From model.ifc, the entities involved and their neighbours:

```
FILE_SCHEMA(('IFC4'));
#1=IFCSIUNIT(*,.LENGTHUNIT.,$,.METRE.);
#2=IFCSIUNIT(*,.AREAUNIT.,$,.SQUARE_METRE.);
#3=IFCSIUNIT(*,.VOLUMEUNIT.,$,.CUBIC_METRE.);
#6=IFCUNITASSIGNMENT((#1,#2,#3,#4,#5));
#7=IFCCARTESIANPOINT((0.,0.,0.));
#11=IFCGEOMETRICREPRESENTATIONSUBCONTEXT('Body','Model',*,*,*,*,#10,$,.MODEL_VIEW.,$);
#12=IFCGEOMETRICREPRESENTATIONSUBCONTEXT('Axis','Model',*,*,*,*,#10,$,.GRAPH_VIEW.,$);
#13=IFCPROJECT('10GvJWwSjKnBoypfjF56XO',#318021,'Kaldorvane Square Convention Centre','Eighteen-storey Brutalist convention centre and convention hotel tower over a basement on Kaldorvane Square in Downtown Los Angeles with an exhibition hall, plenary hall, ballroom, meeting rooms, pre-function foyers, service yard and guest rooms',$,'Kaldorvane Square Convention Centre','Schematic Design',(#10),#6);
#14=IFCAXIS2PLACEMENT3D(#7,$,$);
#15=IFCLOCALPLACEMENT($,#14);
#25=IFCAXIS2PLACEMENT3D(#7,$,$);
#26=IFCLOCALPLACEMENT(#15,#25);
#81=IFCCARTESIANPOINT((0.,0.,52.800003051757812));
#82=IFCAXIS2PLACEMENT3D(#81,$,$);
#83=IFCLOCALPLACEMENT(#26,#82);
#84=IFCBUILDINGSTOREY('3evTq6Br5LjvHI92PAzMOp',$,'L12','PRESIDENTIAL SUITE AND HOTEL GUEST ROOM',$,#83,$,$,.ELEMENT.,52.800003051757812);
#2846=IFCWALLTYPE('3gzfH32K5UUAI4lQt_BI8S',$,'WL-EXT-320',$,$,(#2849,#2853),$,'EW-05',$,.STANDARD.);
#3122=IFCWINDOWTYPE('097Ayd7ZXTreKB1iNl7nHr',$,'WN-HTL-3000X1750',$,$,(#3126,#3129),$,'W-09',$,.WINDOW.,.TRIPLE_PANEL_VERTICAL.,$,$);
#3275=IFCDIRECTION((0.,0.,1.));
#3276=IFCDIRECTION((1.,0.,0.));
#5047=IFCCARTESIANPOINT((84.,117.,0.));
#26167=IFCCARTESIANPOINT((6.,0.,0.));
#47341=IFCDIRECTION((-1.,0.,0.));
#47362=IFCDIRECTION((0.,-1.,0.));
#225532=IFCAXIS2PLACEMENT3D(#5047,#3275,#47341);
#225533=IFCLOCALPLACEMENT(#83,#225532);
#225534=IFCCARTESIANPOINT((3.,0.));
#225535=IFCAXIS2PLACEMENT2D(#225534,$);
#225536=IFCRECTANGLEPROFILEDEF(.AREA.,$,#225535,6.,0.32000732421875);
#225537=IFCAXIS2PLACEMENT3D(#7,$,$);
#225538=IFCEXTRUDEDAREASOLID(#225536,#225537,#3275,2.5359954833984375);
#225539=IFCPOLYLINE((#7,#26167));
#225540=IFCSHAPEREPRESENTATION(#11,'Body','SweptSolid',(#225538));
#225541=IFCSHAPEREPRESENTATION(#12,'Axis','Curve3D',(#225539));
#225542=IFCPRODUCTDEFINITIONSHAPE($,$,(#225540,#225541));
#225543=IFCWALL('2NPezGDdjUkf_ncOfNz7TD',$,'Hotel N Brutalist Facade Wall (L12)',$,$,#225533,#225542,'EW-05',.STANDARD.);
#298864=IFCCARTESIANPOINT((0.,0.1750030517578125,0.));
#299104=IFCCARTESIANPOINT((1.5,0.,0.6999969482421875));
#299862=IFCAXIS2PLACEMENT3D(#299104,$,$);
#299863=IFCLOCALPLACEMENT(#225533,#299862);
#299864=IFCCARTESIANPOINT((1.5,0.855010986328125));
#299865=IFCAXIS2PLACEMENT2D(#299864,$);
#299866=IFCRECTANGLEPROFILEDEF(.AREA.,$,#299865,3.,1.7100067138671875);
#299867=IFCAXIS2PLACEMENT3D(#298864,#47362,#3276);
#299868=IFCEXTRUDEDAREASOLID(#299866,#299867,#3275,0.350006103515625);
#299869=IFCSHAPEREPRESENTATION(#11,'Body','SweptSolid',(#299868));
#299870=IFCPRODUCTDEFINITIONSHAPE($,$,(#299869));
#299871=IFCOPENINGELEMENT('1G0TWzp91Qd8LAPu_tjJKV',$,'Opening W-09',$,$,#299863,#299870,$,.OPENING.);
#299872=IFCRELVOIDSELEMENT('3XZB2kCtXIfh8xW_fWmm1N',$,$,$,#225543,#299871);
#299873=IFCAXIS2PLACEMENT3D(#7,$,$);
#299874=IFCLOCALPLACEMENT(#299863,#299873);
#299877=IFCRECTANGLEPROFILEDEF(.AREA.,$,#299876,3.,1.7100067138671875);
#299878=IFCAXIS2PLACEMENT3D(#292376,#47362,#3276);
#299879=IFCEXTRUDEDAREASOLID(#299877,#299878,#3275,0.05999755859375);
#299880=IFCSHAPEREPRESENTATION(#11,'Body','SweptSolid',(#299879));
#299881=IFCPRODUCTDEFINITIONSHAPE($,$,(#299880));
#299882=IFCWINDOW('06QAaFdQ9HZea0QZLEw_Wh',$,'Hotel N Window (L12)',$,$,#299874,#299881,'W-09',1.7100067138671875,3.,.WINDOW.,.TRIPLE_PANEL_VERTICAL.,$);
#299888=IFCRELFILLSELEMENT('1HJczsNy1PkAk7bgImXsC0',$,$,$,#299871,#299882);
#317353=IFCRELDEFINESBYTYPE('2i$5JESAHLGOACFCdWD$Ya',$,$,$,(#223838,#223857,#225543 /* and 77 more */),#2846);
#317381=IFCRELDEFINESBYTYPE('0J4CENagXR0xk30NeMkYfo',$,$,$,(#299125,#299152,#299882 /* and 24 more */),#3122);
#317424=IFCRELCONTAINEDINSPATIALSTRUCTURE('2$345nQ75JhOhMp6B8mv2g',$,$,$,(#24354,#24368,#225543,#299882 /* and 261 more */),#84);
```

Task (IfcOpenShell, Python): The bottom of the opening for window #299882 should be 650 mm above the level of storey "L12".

```python
import numpy as np
import ifcopenshell
import ifcopenshell.api.geometry
import ifcopenshell.geom
import ifcopenshell.util.element
import ifcopenshell.util.placement
import ifcopenshell.util.shape
import ifcopenshell.util.unit

model = ifcopenshell.open("model.ifc")
unit_scale = ifcopenshell.util.unit.calculate_unit_scale(model)

window = model.by_id(299882)
opening = window.FillsVoids[0].RelatingOpeningElement
storey = ifcopenshell.util.element.get_container(window, ifc_class="IfcBuildingStorey")
level = ifcopenshell.util.placement.get_local_placement(storey.ObjectPlacement)[2, 3]

# The opening's origin need not be at the sill, so measure its lowest point.
shape = ifcopenshell.geom.create_shape(ifcopenshell.geom.settings(), opening)
bottom = ifcopenshell.util.shape.get_shape_bottom_elevation(shape, shape.geometry) / unit_scale
dz = level + 0.65 / unit_scale - bottom

shift = np.array([0.0, 0.0, dz])
# The window is placed relative to its opening, so it follows when the opening moves.
matrix = ifcopenshell.util.placement.get_local_placement(opening.ObjectPlacement)
matrix[:3, 3] += shift
ifcopenshell.api.geometry.edit_object_placement(
    model, product=opening, matrix=matrix, is_si=False, should_transform_children=True
)

print(f"moved by {dz * unit_scale:+.3f} m")

model.write("model-out.ifc")
```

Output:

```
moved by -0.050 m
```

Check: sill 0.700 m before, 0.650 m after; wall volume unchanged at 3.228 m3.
